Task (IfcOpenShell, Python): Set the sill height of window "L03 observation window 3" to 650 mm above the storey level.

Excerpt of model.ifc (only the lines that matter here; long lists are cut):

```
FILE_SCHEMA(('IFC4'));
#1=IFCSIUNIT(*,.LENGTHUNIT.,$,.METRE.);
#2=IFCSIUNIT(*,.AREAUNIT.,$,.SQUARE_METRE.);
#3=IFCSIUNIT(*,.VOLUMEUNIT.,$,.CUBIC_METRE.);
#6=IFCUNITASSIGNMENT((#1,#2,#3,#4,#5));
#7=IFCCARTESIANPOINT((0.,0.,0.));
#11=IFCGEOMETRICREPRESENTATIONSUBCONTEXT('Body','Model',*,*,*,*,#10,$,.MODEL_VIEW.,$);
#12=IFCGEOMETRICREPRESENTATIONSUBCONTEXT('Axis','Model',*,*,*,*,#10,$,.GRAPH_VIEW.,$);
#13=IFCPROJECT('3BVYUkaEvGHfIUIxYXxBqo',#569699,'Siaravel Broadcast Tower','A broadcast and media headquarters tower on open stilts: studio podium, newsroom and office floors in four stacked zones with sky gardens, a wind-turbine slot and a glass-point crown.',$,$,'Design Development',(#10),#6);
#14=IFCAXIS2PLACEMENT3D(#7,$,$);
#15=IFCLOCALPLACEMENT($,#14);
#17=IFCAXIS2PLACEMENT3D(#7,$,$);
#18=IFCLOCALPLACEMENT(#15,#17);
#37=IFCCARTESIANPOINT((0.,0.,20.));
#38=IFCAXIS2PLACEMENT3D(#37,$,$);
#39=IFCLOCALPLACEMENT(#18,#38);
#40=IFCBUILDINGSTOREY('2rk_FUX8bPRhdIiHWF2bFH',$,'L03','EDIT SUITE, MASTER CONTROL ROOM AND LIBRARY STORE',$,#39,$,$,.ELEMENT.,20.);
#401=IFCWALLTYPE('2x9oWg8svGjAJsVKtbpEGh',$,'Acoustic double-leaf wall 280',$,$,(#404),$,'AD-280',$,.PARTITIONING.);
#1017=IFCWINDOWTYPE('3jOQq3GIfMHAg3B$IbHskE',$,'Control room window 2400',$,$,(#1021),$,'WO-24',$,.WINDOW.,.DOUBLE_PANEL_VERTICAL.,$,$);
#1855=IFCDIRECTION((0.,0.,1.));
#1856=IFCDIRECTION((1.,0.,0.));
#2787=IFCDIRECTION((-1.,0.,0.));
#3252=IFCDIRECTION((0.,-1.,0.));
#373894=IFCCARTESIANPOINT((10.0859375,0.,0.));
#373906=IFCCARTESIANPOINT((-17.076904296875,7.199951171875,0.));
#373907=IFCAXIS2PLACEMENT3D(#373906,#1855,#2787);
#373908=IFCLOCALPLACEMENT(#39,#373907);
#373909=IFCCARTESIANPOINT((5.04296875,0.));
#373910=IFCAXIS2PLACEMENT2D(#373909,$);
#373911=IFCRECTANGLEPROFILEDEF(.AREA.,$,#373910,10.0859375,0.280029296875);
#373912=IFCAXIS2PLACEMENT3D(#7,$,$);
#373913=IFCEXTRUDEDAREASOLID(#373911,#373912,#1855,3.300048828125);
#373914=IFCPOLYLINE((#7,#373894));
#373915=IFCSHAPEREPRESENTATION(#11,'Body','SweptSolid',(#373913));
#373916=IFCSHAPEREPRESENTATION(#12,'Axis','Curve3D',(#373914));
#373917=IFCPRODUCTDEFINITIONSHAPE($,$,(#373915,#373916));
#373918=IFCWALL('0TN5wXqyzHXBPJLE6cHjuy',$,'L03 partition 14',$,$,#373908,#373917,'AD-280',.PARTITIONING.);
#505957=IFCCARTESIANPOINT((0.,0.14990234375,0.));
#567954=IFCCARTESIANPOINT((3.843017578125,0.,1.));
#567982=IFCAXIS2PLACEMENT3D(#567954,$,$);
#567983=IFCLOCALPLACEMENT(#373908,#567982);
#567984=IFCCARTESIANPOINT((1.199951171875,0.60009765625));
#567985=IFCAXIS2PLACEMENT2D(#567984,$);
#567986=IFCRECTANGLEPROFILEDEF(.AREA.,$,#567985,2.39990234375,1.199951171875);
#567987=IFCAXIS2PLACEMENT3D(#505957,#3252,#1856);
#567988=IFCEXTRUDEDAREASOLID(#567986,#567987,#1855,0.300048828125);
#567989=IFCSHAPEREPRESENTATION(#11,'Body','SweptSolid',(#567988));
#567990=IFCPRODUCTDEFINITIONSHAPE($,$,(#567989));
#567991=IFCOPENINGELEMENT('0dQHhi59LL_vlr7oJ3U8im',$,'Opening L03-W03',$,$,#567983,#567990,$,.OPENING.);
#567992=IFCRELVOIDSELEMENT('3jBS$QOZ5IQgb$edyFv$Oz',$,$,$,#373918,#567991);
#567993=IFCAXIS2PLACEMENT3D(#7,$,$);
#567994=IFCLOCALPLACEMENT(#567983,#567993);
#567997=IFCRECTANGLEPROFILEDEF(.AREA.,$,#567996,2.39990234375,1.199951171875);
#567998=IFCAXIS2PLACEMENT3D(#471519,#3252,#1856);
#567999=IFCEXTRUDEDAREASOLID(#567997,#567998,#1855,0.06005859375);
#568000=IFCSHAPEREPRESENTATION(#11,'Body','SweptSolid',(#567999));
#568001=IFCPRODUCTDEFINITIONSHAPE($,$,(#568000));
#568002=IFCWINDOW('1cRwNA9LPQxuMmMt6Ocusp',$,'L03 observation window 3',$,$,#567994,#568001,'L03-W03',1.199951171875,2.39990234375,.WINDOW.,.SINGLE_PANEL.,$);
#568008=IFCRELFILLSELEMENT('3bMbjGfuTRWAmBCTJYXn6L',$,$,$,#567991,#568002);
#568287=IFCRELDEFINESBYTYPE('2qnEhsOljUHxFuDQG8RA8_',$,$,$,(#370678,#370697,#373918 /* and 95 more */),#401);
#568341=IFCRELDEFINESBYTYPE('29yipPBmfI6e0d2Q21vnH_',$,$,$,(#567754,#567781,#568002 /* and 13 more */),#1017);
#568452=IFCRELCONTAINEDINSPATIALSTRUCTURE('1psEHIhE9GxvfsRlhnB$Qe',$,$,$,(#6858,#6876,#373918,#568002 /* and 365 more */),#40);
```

```python
import numpy as np
import ifcopenshell
import ifcopenshell.api.geometry
import ifcopenshell.geom
import ifcopenshell.util.element
import ifcopenshell.util.placement
import ifcopenshell.util.shape
import ifcopenshell.util.unit

model = ifcopenshell.open("model.ifc")
unit_scale = ifcopenshell.util.unit.calculate_unit_scale(model)

window = model.by_guid("1cRwNA9LPQxuMmMt6Ocusp")
opening = window.FillsVoids[0].RelatingOpeningElement
storey = ifcopenshell.util.element.get_container(window, ifc_class="IfcBuildingStorey")
level = ifcopenshell.util.placement.get_local_placement(storey.ObjectPlacement)[2, 3]

# The opening's origin need not be at the sill, so measure its lowest point.
shape = ifcopenshell.geom.create_shape(ifcopenshell.geom.settings(), opening)
bottom = ifcopenshell.util.shape.get_shape_bottom_elevation(shape, shape.geometry) / unit_scale
dz = level + 0.65 / unit_scale - bottom

shift = np.array([0.0, 0.0, dz])
# The window is placed relative to its opening, so it follows when the opening moves.
matrix = ifcopenshell.util.placement.get_local_placement(opening.ObjectPlacement)
matrix[:3, 3] += shift
ifcopenshell.api.geometry.edit_object_placement(
    model, product=opening, matrix=matrix, is_si=False, should_transform_children=True
)

print(f"moved by {dz * unit_scale:+.3f} m")

model.write("model_edited.ifc")
```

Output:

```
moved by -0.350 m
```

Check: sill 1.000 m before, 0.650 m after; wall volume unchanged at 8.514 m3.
